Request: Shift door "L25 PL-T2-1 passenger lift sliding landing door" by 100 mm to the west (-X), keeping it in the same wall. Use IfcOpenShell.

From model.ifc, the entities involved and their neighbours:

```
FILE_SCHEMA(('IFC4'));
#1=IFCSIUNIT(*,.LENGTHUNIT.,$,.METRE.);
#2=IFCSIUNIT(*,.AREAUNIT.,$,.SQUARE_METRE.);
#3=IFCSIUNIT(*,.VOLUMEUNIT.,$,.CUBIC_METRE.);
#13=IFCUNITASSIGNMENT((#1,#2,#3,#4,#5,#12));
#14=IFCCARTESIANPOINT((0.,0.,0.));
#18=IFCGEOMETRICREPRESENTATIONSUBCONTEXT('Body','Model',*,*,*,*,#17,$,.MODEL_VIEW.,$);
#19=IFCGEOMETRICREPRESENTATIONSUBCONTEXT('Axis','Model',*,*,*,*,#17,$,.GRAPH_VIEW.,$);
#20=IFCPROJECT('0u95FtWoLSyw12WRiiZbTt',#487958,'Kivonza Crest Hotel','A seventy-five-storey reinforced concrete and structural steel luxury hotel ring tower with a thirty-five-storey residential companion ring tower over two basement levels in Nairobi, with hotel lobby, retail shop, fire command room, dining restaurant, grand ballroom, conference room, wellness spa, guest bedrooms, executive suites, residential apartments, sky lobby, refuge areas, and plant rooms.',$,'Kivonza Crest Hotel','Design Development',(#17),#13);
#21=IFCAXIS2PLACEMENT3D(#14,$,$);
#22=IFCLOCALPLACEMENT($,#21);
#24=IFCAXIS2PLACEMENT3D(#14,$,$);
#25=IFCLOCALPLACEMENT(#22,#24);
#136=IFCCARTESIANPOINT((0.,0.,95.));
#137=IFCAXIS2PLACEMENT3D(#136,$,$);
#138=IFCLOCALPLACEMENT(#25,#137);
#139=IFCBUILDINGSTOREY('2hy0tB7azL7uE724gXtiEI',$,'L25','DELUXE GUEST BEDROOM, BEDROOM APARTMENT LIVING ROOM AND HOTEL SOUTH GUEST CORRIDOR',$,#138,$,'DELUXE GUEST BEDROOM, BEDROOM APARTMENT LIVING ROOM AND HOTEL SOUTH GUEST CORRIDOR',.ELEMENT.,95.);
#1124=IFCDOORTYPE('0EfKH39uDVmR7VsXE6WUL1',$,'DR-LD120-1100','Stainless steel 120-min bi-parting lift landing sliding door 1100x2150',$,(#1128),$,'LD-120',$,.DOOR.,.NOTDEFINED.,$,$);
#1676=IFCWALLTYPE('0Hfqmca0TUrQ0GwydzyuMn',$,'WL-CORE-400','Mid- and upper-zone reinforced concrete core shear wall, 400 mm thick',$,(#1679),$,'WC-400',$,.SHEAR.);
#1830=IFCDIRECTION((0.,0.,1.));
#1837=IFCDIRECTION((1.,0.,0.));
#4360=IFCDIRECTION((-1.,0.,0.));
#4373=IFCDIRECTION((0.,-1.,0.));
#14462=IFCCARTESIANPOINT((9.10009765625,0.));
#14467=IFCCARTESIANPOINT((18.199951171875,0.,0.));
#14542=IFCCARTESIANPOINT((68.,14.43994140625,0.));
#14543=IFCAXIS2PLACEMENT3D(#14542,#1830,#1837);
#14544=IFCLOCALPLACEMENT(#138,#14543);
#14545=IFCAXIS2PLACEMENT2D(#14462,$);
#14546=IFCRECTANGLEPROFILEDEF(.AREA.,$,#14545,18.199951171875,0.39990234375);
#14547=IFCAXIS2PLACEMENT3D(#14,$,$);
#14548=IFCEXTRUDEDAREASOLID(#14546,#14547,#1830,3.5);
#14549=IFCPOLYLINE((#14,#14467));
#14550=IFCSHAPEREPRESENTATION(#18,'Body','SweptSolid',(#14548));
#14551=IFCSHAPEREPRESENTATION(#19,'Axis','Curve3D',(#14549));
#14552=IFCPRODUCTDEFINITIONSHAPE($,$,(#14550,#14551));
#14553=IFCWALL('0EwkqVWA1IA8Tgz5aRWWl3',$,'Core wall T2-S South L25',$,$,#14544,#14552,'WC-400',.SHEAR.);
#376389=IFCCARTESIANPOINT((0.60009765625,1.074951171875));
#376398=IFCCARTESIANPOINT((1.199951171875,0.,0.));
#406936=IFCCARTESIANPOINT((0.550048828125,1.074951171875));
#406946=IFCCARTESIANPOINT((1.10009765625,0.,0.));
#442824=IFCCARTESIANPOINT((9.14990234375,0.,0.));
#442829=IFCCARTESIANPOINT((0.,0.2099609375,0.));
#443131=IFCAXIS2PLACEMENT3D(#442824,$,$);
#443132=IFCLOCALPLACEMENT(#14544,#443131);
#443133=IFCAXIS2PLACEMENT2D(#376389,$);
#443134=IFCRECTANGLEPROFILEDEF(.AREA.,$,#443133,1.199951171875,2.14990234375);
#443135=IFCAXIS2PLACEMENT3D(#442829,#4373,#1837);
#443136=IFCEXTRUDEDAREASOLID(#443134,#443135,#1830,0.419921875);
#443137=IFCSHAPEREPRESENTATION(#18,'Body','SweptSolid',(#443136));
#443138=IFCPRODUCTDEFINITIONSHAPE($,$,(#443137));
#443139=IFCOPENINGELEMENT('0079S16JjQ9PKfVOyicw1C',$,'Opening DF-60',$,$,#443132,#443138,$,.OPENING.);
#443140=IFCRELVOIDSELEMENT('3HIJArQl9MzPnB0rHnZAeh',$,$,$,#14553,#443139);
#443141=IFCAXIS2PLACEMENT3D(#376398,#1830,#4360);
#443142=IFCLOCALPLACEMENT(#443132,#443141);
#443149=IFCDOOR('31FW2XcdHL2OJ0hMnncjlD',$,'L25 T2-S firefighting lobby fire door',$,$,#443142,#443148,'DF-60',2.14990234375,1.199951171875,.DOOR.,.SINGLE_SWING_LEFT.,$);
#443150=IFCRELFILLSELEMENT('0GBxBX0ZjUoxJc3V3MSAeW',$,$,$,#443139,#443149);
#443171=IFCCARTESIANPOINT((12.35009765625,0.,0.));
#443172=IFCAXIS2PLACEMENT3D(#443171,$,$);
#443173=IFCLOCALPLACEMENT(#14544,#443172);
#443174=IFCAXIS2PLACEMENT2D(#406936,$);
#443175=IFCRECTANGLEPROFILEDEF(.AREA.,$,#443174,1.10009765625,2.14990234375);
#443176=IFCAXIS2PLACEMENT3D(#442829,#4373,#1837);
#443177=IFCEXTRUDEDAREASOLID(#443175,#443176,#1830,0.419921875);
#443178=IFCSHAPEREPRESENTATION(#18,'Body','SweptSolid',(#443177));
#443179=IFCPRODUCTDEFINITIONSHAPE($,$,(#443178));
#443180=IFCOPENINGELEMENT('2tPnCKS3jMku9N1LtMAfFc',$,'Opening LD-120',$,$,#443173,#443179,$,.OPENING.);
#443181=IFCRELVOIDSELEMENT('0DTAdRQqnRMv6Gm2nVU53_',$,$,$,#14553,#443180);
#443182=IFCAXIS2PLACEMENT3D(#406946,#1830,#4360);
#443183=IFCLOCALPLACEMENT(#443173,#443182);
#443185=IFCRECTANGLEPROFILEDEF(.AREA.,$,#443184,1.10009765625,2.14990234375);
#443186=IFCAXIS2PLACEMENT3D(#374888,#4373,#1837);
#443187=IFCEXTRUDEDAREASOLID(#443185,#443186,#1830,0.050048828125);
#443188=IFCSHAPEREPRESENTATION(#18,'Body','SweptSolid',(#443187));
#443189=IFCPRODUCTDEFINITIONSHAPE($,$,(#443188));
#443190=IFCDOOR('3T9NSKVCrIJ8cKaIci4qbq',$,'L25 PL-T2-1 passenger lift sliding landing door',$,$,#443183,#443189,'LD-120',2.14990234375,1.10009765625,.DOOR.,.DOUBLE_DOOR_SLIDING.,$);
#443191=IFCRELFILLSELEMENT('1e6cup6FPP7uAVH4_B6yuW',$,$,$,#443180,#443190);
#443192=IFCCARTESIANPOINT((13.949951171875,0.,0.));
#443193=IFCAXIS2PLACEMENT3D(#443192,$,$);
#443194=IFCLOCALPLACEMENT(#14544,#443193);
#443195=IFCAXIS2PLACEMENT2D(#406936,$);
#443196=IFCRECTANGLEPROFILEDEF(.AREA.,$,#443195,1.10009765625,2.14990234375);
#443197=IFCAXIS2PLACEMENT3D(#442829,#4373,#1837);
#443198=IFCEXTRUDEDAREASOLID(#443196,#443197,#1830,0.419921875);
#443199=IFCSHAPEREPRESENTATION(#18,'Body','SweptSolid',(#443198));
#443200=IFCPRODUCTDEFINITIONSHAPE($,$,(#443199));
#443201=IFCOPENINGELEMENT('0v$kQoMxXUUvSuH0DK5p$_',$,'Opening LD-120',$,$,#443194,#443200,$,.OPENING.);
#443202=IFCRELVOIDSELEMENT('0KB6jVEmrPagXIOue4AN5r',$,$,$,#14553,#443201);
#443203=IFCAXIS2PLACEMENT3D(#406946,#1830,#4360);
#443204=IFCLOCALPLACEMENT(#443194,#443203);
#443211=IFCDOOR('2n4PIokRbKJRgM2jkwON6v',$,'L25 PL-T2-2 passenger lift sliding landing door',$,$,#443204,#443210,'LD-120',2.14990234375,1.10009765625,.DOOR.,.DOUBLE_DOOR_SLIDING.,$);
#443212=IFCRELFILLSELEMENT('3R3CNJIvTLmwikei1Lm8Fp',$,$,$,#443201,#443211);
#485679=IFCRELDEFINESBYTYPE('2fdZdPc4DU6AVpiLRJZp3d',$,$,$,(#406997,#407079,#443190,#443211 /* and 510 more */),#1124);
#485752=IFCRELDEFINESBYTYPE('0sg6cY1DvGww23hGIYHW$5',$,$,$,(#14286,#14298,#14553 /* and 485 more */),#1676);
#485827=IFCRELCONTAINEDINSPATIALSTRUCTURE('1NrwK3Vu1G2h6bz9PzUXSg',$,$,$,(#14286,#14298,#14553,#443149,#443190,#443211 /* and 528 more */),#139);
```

```python
import ifcopenshell
import ifcopenshell.api.geometry
import ifcopenshell.util.placement
import ifcopenshell.util.unit

model = ifcopenshell.open("model.ifc")
unit_scale = ifcopenshell.util.unit.calculate_unit_scale(model)

door = model.by_id(443190)
opening = door.FillsVoids[0].RelatingOpeningElement
wall = opening.VoidsElements[0].RelatingBuildingElement

wall_matrix = ifcopenshell.util.placement.get_local_placement(wall.ObjectPlacement)
shift = wall_matrix[:3, 0] * -0.1 / unit_scale
before = ifcopenshell.util.placement.get_local_placement(door.ObjectPlacement)[:3, 3].copy()

# The door is placed relative to its opening, so it follows when the opening moves.
matrix = ifcopenshell.util.placement.get_local_placement(opening.ObjectPlacement)
matrix[:3, 3] += shift
ifcopenshell.api.geometry.edit_object_placement(
    model, product=opening, matrix=matrix, is_si=False, should_transform_children=True
)

after = ifcopenshell.util.placement.get_local_placement(door.ObjectPlacement)[:3, 3]
print("door moved by", (after - before).round(3) + 0.0)

model.write("model-out.ifc")
```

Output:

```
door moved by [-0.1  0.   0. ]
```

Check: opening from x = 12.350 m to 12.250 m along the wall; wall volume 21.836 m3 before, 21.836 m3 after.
